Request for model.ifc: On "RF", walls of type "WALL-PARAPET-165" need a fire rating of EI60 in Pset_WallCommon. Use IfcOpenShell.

First a look at what the model holds.

```python
import ifcopenshell
import ifcopenshell.util.element

model = ifcopenshell.open("model.ifc")
print(model.schema)
storey = next(s for s in model.by_type("IfcBuildingStorey") if s.Name == "RF")
walls = [e for e in ifcopenshell.util.element.get_decomposition(storey) if e.is_a("IfcWall")]
seen = {}
for e in walls:
    element_type = ifcopenshell.util.element.get_type(e)
    key = (element_type.Name if element_type != e and element_type else None, ifcopenshell.util.element.get_pset(e, "Pset_WallCommon", "FireRating"))
    seen[key] = seen.get(key, 0) + 1
for (name, value), count in sorted(seen.items(), key=str):
    print(count, "x", name, "|", value)
```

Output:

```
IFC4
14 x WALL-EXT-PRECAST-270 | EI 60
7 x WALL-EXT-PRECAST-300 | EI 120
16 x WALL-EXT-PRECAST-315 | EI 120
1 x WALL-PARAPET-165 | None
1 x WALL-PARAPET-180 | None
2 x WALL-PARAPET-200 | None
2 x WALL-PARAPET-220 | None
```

```python
import ifcopenshell
import ifcopenshell.api.pset
import ifcopenshell.util.element

model = ifcopenshell.open("model.ifc")

storey = next(s for s in model.by_type("IfcBuildingStorey") if s.Name == "RF")
walls = [e for e in ifcopenshell.util.element.get_decomposition(storey) if e.is_a("IfcWall")]

count = 0
for e in walls:
    element_type = ifcopenshell.util.element.get_type(e)
    if element_type in (None, e) or element_type.Name != "WALL-PARAPET-165":
        continue
    # add_pset returns the element's existing set when there is one.
    pset = ifcopenshell.api.pset.add_pset(model, product=e, name="Pset_WallCommon")
    ifcopenshell.api.pset.edit_pset(model, pset=pset, properties={"FireRating": "EI60"})
    count += 1

print(count, "walls updated")

model.write("model_edited.ifc")
```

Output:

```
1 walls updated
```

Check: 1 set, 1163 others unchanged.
